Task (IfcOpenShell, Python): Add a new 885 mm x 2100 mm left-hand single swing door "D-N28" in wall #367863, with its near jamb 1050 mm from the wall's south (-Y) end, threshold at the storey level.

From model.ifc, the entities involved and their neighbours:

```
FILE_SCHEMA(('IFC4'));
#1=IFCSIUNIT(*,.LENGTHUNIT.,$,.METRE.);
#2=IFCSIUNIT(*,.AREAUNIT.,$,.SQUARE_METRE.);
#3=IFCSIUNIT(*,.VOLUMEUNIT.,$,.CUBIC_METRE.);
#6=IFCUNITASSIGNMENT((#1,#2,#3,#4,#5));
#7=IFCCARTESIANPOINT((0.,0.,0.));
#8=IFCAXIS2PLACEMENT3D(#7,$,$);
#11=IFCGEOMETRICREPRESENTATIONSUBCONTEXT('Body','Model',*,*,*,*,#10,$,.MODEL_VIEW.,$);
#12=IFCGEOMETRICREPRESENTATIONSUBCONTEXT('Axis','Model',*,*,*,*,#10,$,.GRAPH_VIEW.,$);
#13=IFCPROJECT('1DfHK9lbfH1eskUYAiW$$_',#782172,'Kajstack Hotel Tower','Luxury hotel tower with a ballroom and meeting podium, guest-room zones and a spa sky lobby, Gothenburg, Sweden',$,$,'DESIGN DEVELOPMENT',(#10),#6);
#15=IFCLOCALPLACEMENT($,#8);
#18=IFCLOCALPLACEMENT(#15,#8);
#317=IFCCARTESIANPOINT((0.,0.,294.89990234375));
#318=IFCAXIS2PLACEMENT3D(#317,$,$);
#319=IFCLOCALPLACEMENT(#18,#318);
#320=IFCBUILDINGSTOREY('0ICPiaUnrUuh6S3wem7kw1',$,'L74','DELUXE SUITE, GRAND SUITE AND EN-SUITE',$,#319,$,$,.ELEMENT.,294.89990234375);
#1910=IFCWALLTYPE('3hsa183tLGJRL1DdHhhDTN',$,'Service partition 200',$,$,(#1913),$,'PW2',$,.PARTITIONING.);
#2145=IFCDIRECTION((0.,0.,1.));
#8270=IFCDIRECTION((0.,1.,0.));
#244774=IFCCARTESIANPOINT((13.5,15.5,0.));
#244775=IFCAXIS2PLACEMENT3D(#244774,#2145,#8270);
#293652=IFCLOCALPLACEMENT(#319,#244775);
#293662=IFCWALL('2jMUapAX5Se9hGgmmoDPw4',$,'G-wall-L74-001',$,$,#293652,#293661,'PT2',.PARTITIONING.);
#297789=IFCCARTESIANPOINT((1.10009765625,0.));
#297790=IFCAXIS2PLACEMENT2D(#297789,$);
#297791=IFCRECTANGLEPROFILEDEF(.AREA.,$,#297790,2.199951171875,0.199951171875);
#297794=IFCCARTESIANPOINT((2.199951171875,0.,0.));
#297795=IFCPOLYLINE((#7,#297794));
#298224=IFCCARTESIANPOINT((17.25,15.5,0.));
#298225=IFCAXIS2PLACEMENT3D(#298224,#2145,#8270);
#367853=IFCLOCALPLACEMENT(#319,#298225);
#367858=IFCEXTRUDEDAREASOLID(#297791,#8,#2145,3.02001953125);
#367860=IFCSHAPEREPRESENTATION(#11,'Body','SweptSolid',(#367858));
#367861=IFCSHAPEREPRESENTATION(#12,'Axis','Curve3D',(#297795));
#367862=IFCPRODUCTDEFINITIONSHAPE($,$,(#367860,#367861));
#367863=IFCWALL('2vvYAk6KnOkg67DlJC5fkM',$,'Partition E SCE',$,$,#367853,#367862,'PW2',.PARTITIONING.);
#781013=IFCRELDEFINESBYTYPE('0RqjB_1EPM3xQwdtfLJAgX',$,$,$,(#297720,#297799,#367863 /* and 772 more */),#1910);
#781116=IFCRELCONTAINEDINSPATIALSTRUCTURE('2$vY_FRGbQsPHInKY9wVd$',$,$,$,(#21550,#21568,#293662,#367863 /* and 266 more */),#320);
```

```python
import numpy as np
import ifcopenshell
import ifcopenshell.api.feature
import ifcopenshell.api.geometry
import ifcopenshell.api.root
import ifcopenshell.api.spatial
import ifcopenshell.geom
import ifcopenshell.util.element
import ifcopenshell.util.placement
import ifcopenshell.util.representation
import ifcopenshell.util.shape
import ifcopenshell.util.unit

model = ifcopenshell.open("model.ifc")
unit_scale = ifcopenshell.util.unit.calculate_unit_scale(model)
settings = ifcopenshell.geom.settings()


def volume(element):
    """Net volume in cubic metres, openings subtracted."""
    shape = ifcopenshell.geom.create_shape(settings, element)
    return ifcopenshell.util.shape.get_volume(shape.geometry)


wall = model.by_guid("2vvYAk6KnOkg67DlJC5fkM")
storey = ifcopenshell.util.element.get_container(wall, ifc_class="IfcBuildingStorey")
context = ifcopenshell.util.representation.get_context(model, "Model", "Body", "MODEL_VIEW")
before = volume(wall)

width, height, from_end, sill = 0.885, 2.1, 1.05, 0.0  # metres

# The wall runs along its own X axis, and the end named is its -X end.
wall_shape = ifcopenshell.geom.create_shape(settings, wall)
x, y, z = ifcopenshell.util.shape.get_vertices(wall_shape.geometry).T
start = x.min() + from_end
face, thickness = float(y.min()), float(y.max() - y.min())
wall_matrix = ifcopenshell.util.placement.get_local_placement(wall.ObjectPlacement)
level = ifcopenshell.util.placement.get_local_placement(storey.ObjectPlacement)[2, 3]


def in_wall(x, y):
    """Placement at x, y metres in the wall's axes, at sill height."""
    matrix = wall_matrix.copy()
    matrix[:, 3] = wall_matrix @ np.array([x / unit_scale, y / unit_scale, 0.0, 1.0])
    matrix[2, 3] = level + sill / unit_scale
    return matrix


# Opening: a box that overshoots both wall faces by 50 mm.
opening = ifcopenshell.api.root.create_entity(model, ifc_class="IfcOpeningElement", predefined_type="OPENING")
box = ifcopenshell.api.geometry.add_wall_representation(
    model, context=context, length=width, height=height, thickness=thickness + 0.1
)
ifcopenshell.api.geometry.assign_representation(model, product=opening, representation=box)
ifcopenshell.api.geometry.edit_object_placement(model, product=opening, matrix=in_wall(start, face - 0.05), is_si=False)
ifcopenshell.api.feature.add_feature(model, feature=opening, element=wall)

door = ifcopenshell.api.root.create_entity(model, ifc_class="IfcDoor", name="D-N28", predefined_type="DOOR")
door.OverallWidth, door.OverallHeight = width / unit_scale, height / unit_scale
door.OperationType = "SINGLE_SWING_LEFT"
body = ifcopenshell.api.geometry.add_door_representation(
    model,
    context=context,
    overall_width=door.OverallWidth,
    overall_height=door.OverallHeight,
    operation_type="SINGLE_SWING_LEFT",
    lining_properties={"LiningDepth": thickness / unit_scale, "ThresholdDepth": thickness / unit_scale},
)
ifcopenshell.api.geometry.assign_representation(model, product=door, representation=body)
ifcopenshell.api.spatial.assign_container(model, products=[door], relating_structure=storey)
ifcopenshell.api.feature.add_filling(model, opening=opening, element=door)

# The lining spans the wall, so the door starts at the wall face.
ifcopenshell.api.geometry.edit_object_placement(model, product=door, matrix=in_wall(start, face), is_si=False)

after = volume(wall)

print(f"wall volume {before:.3f} -> {after:.3f} m3")

model.write("model-out.ifc")
```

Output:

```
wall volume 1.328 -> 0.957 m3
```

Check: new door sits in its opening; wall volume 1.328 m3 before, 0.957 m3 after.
